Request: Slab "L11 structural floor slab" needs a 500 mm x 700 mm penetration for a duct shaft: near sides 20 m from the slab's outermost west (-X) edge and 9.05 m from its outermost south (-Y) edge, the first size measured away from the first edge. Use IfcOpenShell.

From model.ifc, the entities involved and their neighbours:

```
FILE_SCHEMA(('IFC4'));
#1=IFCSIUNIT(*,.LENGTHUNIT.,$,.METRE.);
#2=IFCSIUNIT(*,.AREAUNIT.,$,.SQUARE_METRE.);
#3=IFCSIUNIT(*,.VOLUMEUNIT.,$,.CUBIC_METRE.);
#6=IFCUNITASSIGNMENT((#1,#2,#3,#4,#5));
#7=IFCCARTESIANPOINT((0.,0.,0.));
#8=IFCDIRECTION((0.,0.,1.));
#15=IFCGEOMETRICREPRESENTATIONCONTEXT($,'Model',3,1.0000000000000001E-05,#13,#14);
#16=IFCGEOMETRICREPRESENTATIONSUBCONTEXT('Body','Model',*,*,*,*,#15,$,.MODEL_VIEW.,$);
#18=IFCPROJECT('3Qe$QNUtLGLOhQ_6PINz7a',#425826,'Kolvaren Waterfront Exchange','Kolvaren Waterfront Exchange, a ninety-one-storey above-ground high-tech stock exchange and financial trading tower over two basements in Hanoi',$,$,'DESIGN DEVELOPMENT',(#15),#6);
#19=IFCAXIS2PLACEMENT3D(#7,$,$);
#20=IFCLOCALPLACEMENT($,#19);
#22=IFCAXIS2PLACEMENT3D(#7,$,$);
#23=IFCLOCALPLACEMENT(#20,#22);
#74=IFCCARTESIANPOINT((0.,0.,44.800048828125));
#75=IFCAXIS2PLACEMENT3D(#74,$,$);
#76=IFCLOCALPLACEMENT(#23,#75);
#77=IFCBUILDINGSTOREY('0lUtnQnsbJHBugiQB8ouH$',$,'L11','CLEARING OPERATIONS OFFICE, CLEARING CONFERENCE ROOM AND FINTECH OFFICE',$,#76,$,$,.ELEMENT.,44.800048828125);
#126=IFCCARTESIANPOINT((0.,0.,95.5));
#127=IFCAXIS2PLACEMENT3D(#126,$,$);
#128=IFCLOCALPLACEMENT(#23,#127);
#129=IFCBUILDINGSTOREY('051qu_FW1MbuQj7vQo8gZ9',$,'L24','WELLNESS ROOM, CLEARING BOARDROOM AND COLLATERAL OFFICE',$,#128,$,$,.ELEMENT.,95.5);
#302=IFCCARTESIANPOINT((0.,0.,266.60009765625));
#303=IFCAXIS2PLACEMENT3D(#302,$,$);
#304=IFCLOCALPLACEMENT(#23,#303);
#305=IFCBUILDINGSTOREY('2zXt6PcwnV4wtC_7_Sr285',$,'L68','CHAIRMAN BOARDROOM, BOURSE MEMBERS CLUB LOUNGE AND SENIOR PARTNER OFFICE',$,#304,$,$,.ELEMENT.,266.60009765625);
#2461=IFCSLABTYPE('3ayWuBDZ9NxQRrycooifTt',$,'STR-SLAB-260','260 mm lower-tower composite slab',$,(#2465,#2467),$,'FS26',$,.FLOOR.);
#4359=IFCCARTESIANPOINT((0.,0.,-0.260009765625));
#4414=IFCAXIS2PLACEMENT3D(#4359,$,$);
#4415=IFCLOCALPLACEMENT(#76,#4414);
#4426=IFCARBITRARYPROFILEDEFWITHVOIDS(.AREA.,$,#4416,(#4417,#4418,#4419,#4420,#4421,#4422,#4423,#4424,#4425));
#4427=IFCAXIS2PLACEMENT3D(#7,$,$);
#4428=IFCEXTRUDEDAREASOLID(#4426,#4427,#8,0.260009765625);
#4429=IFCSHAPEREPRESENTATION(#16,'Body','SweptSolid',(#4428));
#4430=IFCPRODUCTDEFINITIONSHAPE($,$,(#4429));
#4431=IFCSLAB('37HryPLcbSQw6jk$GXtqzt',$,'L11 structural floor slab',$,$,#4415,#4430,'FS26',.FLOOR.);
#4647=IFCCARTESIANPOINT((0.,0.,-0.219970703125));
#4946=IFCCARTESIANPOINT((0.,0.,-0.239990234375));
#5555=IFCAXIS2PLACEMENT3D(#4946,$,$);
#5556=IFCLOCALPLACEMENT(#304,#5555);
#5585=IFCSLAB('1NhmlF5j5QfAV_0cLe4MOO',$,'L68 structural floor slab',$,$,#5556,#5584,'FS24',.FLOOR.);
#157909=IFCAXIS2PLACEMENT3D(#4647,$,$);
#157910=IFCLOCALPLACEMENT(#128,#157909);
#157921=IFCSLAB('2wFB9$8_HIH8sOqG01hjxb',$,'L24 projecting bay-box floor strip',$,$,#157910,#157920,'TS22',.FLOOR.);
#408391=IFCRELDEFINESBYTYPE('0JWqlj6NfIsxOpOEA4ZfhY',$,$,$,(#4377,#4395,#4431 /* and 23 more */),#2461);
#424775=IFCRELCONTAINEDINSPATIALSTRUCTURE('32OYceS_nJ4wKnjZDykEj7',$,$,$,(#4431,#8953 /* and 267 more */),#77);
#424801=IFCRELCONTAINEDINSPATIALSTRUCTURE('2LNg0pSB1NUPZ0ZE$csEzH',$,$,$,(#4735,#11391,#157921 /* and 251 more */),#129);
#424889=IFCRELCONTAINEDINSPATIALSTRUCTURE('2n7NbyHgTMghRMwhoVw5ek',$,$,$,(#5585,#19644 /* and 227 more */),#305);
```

```python
import numpy as np
import ifcopenshell
import ifcopenshell.api.feature
import ifcopenshell.api.geometry
import ifcopenshell.api.root
import ifcopenshell.geom
import ifcopenshell.util.placement
import ifcopenshell.util.representation
import ifcopenshell.util.shape
import ifcopenshell.util.unit

model = ifcopenshell.open("model.ifc")
unit_scale = ifcopenshell.util.unit.calculate_unit_scale(model)
settings = ifcopenshell.geom.settings()


def volume(element):
    """Net volume in cubic metres, openings subtracted."""
    shape = ifcopenshell.geom.create_shape(settings, element)
    return ifcopenshell.util.shape.get_volume(shape.geometry)


slab = model.by_guid("37HryPLcbSQw6jk$GXtqzt")
before = volume(slab)

# Extent in the slab's own axes, in metres. The edges named are its -X and -Y sides.
slab_shape = ifcopenshell.geom.create_shape(settings, slab)
vertices = ifcopenshell.util.shape.get_vertices(slab_shape.geometry)
x_min, y_min, bottom = vertices.min(axis=0)
top = vertices[:, 2].max()

opening = ifcopenshell.api.root.create_entity(model, ifc_class="IfcOpeningElement", name="Duct shaft opening", predefined_type="OPENING")
context = ifcopenshell.util.representation.get_context(model, "Model", "Body", "MODEL_VIEW")
width, depth = 0.5, 0.7
outline = [(0.0, 0.0), (width, 0.0), (width, depth), (0.0, depth), (0.0, 0.0)]
# Overshoot both faces by 50 mm so the cut is clean.
shape = ifcopenshell.api.geometry.add_slab_representation(
    model, context=context, depth=top - bottom + 0.1, polyline=outline
)
ifcopenshell.api.geometry.assign_representation(model, product=opening, representation=shape)

matrix = ifcopenshell.util.placement.get_local_placement(slab.ObjectPlacement)
matrix[:, 3] = matrix @ np.append(np.array([x_min + 20, y_min + 9.05, bottom - 0.05]) / unit_scale, 1.0)
ifcopenshell.api.geometry.edit_object_placement(model, product=opening, matrix=matrix, is_si=False)
ifcopenshell.api.feature.add_feature(model, feature=opening, element=slab)

after = volume(slab)

print(f"slab volume {before:.3f} -> {after:.3f} m3")

model.write("model-out.ifc")
```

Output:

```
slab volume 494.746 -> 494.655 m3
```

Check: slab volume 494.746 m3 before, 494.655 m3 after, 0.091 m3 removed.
